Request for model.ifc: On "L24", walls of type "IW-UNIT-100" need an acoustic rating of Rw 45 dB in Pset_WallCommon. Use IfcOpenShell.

First a look at what the model holds.

```python
import ifcopenshell
import ifcopenshell.util.element

model = ifcopenshell.open("model.ifc")
print(model.schema)
storey = next(s for s in model.by_type("IfcBuildingStorey") if s.Name == "L24")
walls = [e for e in ifcopenshell.util.element.get_decomposition(storey) if e.is_a("IfcWall")]
seen = {}
for e in walls:
    element_type = ifcopenshell.util.element.get_type(e)
    key = (element_type.Name if element_type != e and element_type else None, ifcopenshell.util.element.get_pset(e, "Pset_WallCommon", "AcousticRating"))
    seen[key] = seen.get(key, 0) + 1
for (name, value), count in sorted(seen.items(), key=str):
    print(count, "x", name, "|", value)
```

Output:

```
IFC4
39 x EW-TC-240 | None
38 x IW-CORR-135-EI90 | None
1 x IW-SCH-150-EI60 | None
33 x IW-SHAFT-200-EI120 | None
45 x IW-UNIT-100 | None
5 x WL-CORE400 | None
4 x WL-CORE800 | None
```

```python
import ifcopenshell
import ifcopenshell.api.pset
import ifcopenshell.util.element

model = ifcopenshell.open("model.ifc")

storey = next(s for s in model.by_type("IfcBuildingStorey") if s.Name == "L24")
walls = [e for e in ifcopenshell.util.element.get_decomposition(storey) if e.is_a("IfcWall")]

count = 0
for e in walls:
    element_type = ifcopenshell.util.element.get_type(e)
    if element_type in (None, e) or element_type.Name != "IW-UNIT-100":
        continue
    found = ifcopenshell.util.element.get_pset(e, "Pset_WallCommon", should_inherit=False)
    if found:
        pset = model.by_id(found["id"])
        if len(ifcopenshell.util.element.get_elements_by_pset(pset)) > 1:
            pset = ifcopenshell.api.pset.unshare_pset(model, products=[e], pset=pset)[0]
    else:
        pset = ifcopenshell.api.pset.add_pset(model, product=e, name="Pset_WallCommon")
    ifcopenshell.api.pset.edit_pset(model, pset=pset, properties={"AcousticRating": "Rw 45 dB"})
    count += 1

print(count, "walls updated")

model.write("model-out.ifc")
```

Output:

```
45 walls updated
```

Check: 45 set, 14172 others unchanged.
